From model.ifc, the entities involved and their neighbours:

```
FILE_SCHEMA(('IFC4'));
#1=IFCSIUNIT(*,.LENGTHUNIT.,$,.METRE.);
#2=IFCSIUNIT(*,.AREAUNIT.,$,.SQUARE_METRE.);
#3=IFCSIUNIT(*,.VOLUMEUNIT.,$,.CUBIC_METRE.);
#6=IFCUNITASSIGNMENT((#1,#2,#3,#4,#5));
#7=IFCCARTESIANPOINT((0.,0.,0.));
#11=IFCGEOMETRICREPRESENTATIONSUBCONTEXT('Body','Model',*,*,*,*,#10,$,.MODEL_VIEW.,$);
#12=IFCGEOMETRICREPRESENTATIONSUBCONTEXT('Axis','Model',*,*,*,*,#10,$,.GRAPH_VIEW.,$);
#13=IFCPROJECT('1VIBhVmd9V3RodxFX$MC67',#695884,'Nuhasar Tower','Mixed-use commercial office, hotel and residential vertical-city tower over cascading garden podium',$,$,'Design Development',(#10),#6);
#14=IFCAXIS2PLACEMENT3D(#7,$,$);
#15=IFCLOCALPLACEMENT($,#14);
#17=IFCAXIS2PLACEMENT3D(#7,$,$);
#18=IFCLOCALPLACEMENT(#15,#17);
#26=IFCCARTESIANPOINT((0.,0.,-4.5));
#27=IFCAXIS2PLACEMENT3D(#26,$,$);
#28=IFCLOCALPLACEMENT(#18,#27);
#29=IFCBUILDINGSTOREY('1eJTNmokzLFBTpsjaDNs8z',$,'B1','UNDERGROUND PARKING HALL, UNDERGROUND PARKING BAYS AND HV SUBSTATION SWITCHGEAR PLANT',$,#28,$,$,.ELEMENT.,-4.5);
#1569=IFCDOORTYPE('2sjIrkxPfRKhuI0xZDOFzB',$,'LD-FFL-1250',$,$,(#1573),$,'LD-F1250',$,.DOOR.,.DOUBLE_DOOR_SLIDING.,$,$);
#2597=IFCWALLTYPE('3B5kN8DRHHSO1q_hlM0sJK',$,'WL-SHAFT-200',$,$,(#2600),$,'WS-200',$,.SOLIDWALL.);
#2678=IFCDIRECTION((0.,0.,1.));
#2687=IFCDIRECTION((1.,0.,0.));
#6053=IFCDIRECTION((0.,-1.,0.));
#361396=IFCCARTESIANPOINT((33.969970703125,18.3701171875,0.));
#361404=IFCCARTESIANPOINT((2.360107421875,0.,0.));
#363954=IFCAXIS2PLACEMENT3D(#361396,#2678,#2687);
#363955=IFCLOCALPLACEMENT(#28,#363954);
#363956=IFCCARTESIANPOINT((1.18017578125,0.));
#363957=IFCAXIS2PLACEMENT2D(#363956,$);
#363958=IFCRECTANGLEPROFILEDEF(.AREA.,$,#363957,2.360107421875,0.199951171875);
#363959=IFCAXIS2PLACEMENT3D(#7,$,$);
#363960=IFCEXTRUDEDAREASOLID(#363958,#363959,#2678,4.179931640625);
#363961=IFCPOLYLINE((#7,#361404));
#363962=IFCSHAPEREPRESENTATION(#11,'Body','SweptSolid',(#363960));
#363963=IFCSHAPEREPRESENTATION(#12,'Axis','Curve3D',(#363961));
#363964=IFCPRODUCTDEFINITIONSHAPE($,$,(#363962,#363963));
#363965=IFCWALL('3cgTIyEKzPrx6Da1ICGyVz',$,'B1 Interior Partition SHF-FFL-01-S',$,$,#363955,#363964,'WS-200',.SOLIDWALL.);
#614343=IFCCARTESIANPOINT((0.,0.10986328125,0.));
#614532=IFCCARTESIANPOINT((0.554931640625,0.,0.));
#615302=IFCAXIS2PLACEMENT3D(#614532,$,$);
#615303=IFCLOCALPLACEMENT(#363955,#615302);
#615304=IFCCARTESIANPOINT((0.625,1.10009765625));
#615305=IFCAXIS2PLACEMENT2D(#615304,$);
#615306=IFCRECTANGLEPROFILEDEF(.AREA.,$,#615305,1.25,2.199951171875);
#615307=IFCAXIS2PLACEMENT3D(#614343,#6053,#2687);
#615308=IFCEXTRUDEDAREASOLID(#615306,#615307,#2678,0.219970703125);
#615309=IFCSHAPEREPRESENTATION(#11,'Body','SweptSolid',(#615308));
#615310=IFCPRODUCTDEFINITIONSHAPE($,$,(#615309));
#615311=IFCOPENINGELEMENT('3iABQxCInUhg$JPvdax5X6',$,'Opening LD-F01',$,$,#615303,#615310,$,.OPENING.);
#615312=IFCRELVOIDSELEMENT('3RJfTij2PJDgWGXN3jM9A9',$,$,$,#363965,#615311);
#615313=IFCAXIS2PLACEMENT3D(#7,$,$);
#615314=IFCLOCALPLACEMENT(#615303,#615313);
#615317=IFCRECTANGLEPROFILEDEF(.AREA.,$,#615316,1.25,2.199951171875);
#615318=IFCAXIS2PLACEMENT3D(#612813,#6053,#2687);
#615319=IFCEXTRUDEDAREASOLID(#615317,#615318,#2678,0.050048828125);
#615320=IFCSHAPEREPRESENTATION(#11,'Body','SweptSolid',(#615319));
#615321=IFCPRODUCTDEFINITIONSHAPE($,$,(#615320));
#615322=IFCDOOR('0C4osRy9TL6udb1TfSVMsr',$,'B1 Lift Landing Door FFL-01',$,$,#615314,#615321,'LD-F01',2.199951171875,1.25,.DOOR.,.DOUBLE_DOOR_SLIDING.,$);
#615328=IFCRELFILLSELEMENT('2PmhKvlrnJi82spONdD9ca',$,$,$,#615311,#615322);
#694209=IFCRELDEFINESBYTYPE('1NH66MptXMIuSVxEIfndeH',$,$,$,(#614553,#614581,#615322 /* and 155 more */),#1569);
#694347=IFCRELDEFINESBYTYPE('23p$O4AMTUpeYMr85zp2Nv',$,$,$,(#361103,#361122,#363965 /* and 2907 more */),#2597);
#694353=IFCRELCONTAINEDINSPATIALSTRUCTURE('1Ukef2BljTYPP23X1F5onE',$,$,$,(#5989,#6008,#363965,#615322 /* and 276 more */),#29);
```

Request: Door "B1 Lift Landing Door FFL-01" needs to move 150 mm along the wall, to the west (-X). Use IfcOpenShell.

```python
import ifcopenshell
import ifcopenshell.api.geometry
import ifcopenshell.util.placement

model = ifcopenshell.open("model.ifc")

door = model.by_guid("0C4osRy9TL6udb1TfSVMsr")
opening = door.FillsVoids[0].RelatingOpeningElement
wall = opening.VoidsElements[0].RelatingBuildingElement

wall_matrix = ifcopenshell.util.placement.get_local_placement(wall.ObjectPlacement)
shift = wall_matrix[:3, 0] * -0.15
before = ifcopenshell.util.placement.get_local_placement(door.ObjectPlacement)[:3, 3].copy()

# The door is placed relative to its opening, so it follows when the opening moves.
matrix = ifcopenshell.util.placement.get_local_placement(opening.ObjectPlacement)
matrix[:3, 3] += shift
ifcopenshell.api.geometry.edit_object_placement(
    model, product=opening, matrix=matrix, is_si=False, should_transform_children=True
)

after = ifcopenshell.util.placement.get_local_placement(door.ObjectPlacement)[:3, 3]
print("door moved by", (after - before).round(3) + 0.0)

model.write("model-out.ifc")
```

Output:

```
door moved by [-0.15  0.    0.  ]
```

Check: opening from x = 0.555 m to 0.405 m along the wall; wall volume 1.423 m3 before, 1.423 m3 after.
